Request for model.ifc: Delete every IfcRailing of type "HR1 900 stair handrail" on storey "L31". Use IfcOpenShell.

First a look at what the model holds.

```python
import ifcopenshell
import ifcopenshell.util.element

model = ifcopenshell.open("model.ifc")
print(model.schema)
storey = next(s for s in model.by_type("IfcBuildingStorey") if s.Name == "L31")
railings = [e for e in ifcopenshell.util.element.get_decomposition(storey) if e.is_a("IfcRailing")]
seen = {}
for e in railings:
    element_type = ifcopenshell.util.element.get_type(e)
    name = element_type.Name if element_type not in (None, e) else None
    seen[name] = seen.get(name, 0) + 1
for name, count in sorted(seen.items(), key=str):
    print(count, "x", name)
```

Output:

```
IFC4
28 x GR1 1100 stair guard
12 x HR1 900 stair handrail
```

```python
import ifcopenshell
import ifcopenshell.api.root
import ifcopenshell.util.element

model = ifcopenshell.open("model.ifc")

storey = next(s for s in model.by_type("IfcBuildingStorey") if s.Name == "L31")
railings = [e for e in ifcopenshell.util.element.get_decomposition(storey) if e.is_a("IfcRailing")]
targets = [e for e in railings if (t := ifcopenshell.util.element.get_type(e)) not in (None, e) and t.Name == "HR1 900 stair handrail"]

for e in targets:
    ifcopenshell.api.root.remove_product(model, product=e)
print(len(targets), "removed")

model.write("model-out.ifc")
```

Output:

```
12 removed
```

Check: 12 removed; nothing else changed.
